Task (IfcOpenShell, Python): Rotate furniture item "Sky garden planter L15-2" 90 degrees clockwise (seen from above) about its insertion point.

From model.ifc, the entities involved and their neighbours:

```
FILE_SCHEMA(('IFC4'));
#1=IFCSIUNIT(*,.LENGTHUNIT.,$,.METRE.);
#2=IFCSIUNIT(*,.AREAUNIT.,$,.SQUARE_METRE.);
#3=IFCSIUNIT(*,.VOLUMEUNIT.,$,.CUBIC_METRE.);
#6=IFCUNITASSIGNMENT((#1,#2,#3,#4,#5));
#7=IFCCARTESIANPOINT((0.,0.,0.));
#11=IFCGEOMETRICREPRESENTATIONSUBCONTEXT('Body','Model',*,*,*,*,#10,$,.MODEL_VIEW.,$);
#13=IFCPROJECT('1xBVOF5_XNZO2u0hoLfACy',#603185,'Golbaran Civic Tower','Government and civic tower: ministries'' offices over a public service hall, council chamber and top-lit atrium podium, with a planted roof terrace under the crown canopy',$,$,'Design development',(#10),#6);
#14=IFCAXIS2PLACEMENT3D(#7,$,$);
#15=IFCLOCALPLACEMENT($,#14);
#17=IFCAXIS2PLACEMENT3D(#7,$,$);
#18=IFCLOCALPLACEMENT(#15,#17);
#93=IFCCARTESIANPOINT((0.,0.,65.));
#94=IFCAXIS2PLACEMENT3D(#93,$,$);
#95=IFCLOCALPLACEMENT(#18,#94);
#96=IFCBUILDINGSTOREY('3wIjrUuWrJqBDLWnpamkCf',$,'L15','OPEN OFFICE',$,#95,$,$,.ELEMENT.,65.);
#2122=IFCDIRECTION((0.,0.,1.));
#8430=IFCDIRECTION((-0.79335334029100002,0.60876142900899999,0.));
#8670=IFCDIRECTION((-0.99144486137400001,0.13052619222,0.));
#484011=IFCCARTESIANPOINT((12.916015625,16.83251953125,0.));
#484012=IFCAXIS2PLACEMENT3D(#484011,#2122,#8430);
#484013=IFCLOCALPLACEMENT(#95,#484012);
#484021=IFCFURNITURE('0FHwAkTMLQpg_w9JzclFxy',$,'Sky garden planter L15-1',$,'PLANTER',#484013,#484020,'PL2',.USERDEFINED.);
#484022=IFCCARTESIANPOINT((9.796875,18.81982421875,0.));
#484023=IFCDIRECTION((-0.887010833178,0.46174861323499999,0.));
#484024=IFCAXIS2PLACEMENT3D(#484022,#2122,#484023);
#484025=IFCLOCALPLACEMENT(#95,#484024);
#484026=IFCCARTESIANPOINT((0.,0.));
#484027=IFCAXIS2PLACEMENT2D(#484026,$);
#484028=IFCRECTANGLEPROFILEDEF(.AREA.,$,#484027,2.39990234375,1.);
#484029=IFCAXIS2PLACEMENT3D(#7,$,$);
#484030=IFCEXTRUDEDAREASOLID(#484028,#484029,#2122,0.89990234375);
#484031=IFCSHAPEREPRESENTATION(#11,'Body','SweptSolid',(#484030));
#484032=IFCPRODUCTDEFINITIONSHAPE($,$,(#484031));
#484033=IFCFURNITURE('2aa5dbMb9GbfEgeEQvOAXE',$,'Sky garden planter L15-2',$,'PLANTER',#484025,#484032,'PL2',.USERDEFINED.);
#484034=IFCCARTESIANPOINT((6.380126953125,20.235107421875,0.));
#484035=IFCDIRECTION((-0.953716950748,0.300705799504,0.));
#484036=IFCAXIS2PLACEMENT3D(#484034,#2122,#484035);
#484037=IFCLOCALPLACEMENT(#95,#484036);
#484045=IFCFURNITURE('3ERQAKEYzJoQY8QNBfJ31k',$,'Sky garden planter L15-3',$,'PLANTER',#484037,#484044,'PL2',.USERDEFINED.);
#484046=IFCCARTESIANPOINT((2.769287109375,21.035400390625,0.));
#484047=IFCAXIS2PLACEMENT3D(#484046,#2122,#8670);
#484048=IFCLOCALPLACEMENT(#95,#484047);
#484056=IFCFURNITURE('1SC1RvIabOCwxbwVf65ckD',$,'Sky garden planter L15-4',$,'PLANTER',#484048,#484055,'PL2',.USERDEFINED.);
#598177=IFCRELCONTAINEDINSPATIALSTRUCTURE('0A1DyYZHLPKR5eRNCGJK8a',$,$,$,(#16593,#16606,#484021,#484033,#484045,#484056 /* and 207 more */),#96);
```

```python
import ifcopenshell
import ifcopenshell.api.geometry
import ifcopenshell.util.placement

model = ifcopenshell.open("model.ifc")

item = model.by_id(484033)
matrix = ifcopenshell.util.placement.get_local_placement(item.ObjectPlacement)
matrix = matrix @ ifcopenshell.util.placement.rotation(-90, "Z")
ifcopenshell.api.geometry.edit_object_placement(model, product=item, matrix=matrix, is_si=False)

print(ifcopenshell.util.placement.get_local_placement(item.ObjectPlacement).round(3) + 0.0)

model.write("model_v2.ifc")
```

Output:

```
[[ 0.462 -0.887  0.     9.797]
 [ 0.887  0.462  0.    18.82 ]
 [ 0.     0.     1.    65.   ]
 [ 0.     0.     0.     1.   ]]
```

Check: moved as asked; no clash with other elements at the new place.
